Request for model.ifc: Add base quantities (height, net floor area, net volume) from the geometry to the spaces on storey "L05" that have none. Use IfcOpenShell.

First a look at what the model holds.

```python
import ifcopenshell
import ifcopenshell.util.element
import ifcopenshell.util.unit

model = ifcopenshell.open("model.ifc")
print(model.schema)
for unit_type in ("LENGTHUNIT", "AREAUNIT", "VOLUMEUNIT"):
    print(unit_type, ifcopenshell.util.unit.calculate_unit_scale(model, unit_type))
storey = next(s for s in model.by_type("IfcBuildingStorey") if s.Name == "L05")
spaces = [e for e in ifcopenshell.util.element.get_decomposition(storey) if e.is_a("IfcSpace")]
for e in sorted(spaces, key=lambda e: e.id()):
    print(e.id(), e.is_a(), e.Name, list(ifcopenshell.util.element.get_psets(e, qtos_only=True)), sep=" | ")
```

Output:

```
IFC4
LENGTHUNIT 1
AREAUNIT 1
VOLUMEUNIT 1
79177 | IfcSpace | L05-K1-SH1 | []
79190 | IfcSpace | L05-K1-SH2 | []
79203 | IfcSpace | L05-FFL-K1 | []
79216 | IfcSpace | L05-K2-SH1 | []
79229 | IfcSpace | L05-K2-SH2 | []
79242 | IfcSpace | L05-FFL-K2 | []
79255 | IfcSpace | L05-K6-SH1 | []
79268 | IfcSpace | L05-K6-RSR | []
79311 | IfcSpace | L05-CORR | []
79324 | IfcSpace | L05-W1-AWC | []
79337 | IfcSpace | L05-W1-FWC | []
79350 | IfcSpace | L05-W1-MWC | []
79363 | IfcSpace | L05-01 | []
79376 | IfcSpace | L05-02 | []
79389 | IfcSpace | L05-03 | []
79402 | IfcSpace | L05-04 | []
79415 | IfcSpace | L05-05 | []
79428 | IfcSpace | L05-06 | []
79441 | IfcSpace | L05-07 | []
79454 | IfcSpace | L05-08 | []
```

```python
import ifcopenshell
import ifcopenshell.api.pset
import ifcopenshell.geom
import ifcopenshell.util.element
import ifcopenshell.util.shape
import ifcopenshell.util.unit

model = ifcopenshell.open("model.ifc")
unit_scale = ifcopenshell.util.unit.calculate_unit_scale(model)
area_scale = ifcopenshell.util.unit.calculate_unit_scale(model, "AREAUNIT")
volume_scale = ifcopenshell.util.unit.calculate_unit_scale(model, "VOLUMEUNIT")
settings = ifcopenshell.geom.settings()

storey = next(s for s in model.by_type("IfcBuildingStorey") if s.Name == "L05")
spaces = [e for e in ifcopenshell.util.element.get_decomposition(storey) if e.is_a("IfcSpace")]

for e in sorted(spaces, key=lambda e: e.id()):
    if ifcopenshell.util.element.get_psets(e, qtos_only=True, should_inherit=False):
        continue
    # Geometry comes back in metres, in the element's own axes.
    shape = ifcopenshell.geom.create_shape(settings, e)
    values = {
        "Height": ifcopenshell.util.shape.get_z(shape.geometry) / unit_scale,
        "NetFloorArea": ifcopenshell.util.shape.get_footprint_area(shape.geometry) / area_scale,
        "NetVolume": ifcopenshell.util.shape.get_volume(shape.geometry) / volume_scale,
    }
    qto = ifcopenshell.api.pset.add_qto(model, product=e, name="Qto_SpaceBaseQuantities")
    ifcopenshell.api.pset.edit_qto(model, qto=qto, properties=values)
    print(e.id(), {k: round(v, 3) for k, v in values.items()})

model.write("model_edited.ifc")
```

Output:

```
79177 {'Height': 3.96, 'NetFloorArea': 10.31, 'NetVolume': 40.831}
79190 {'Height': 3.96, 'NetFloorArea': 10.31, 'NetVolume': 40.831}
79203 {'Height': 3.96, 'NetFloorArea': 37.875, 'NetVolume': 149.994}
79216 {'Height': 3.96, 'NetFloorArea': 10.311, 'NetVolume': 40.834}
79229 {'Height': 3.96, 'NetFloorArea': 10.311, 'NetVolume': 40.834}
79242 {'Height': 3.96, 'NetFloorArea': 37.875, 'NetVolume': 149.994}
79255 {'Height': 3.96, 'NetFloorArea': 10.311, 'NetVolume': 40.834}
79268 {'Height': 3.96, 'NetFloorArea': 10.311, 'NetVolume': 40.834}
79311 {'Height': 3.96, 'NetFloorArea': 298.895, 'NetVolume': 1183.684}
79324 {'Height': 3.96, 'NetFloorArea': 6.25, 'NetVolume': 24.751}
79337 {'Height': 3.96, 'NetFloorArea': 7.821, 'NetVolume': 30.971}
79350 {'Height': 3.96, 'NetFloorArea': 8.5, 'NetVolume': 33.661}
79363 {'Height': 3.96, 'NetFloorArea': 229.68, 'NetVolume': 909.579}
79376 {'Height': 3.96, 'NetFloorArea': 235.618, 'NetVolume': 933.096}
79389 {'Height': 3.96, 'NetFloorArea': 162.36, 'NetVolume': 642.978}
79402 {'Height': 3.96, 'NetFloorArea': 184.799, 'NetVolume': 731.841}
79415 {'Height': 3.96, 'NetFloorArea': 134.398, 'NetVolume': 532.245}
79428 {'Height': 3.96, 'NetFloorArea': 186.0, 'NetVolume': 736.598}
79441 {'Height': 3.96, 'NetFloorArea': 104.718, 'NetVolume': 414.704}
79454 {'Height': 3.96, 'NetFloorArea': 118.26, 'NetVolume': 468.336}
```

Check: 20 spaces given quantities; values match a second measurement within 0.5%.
